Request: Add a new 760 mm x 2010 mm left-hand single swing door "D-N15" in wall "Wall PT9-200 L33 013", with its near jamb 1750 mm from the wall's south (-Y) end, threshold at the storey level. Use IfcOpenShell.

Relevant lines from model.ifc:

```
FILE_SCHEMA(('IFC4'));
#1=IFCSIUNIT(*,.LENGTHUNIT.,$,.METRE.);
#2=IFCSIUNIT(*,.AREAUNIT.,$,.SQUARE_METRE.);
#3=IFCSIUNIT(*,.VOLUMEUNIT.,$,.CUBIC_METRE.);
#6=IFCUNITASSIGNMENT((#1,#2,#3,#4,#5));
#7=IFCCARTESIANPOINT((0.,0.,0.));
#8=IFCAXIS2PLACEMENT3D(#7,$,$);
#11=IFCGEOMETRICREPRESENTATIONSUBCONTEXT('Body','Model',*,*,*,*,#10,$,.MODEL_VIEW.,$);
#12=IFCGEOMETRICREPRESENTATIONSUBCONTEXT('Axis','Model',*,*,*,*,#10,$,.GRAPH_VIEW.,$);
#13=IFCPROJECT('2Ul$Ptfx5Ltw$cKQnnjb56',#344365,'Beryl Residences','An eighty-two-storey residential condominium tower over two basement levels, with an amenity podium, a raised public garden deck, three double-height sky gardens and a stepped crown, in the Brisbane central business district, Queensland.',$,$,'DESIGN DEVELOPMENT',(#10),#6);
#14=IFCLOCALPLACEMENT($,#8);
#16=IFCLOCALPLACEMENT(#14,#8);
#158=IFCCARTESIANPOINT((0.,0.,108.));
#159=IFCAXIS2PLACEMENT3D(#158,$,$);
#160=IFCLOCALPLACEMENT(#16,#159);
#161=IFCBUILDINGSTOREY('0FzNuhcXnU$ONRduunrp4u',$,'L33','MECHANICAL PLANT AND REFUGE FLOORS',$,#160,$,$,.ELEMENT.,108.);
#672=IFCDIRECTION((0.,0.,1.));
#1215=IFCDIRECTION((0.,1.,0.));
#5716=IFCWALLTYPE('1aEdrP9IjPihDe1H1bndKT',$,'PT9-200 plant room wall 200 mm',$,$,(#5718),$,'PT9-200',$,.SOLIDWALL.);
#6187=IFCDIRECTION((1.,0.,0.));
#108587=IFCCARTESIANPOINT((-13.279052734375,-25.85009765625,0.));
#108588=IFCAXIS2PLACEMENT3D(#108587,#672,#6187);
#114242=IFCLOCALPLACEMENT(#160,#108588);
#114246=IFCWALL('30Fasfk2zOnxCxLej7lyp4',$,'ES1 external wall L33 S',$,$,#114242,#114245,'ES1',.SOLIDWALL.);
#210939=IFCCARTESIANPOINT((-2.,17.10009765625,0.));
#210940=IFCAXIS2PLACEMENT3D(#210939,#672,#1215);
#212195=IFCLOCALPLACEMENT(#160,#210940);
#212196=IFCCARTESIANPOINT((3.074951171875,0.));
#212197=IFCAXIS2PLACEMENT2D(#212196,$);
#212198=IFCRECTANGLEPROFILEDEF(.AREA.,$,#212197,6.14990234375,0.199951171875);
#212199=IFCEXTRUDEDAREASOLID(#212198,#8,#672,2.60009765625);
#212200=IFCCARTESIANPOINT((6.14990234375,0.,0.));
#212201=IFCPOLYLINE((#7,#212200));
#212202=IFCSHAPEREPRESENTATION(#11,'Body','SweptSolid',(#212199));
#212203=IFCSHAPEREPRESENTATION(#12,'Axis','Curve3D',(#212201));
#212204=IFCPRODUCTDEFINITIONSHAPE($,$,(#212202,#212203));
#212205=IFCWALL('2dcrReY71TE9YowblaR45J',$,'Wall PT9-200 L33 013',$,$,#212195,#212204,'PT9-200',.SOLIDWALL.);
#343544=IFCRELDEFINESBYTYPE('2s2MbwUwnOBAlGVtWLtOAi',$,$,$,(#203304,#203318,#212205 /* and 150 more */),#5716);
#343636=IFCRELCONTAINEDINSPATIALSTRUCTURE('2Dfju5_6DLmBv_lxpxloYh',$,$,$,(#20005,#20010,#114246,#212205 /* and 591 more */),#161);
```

```python
import numpy as np
import ifcopenshell
import ifcopenshell.api.feature
import ifcopenshell.api.geometry
import ifcopenshell.api.root
import ifcopenshell.api.spatial
import ifcopenshell.geom
import ifcopenshell.util.element
import ifcopenshell.util.placement
import ifcopenshell.util.representation
import ifcopenshell.util.shape
import ifcopenshell.util.unit

model = ifcopenshell.open("model.ifc")
unit_scale = ifcopenshell.util.unit.calculate_unit_scale(model)
settings = ifcopenshell.geom.settings()


def volume(element):
    """Net volume in cubic metres, openings subtracted."""
    shape = ifcopenshell.geom.create_shape(settings, element)
    return ifcopenshell.util.shape.get_volume(shape.geometry)


wall = model.by_guid("2dcrReY71TE9YowblaR45J")
storey = ifcopenshell.util.element.get_container(wall, ifc_class="IfcBuildingStorey")
context = ifcopenshell.util.representation.get_context(model, "Model", "Body", "MODEL_VIEW")
before = volume(wall)

width, height, from_end, sill = 0.76, 2.01, 1.75, 0.0  # metres

# The wall runs along its own X axis, and the end named is its -X end.
wall_shape = ifcopenshell.geom.create_shape(settings, wall)
x, y, z = ifcopenshell.util.shape.get_vertices(wall_shape.geometry).T
start = x.min() + from_end
face, thickness = float(y.min()), float(y.max() - y.min())
wall_matrix = ifcopenshell.util.placement.get_local_placement(wall.ObjectPlacement)
level = ifcopenshell.util.placement.get_local_placement(storey.ObjectPlacement)[2, 3]


def in_wall(x, y):
    """Placement at x, y metres in the wall's axes, at sill height."""
    matrix = wall_matrix.copy()
    matrix[:, 3] = wall_matrix @ np.array([x / unit_scale, y / unit_scale, 0.0, 1.0])
    matrix[2, 3] = level + sill / unit_scale
    return matrix


# Opening: a box that overshoots both wall faces by 50 mm.
opening = ifcopenshell.api.root.create_entity(model, ifc_class="IfcOpeningElement", predefined_type="OPENING")
box = ifcopenshell.api.geometry.add_wall_representation(
    model, context=context, length=width, height=height, thickness=thickness + 0.1
)
ifcopenshell.api.geometry.assign_representation(model, product=opening, representation=box)
ifcopenshell.api.geometry.edit_object_placement(model, product=opening, matrix=in_wall(start, face - 0.05), is_si=False)
ifcopenshell.api.feature.add_feature(model, feature=opening, element=wall)

door = ifcopenshell.api.root.create_entity(model, ifc_class="IfcDoor", name="D-N15", predefined_type="DOOR")
door.OverallWidth, door.OverallHeight = width / unit_scale, height / unit_scale
door.OperationType = "SINGLE_SWING_LEFT"
body = ifcopenshell.api.geometry.add_door_representation(
    model,
    context=context,
    overall_width=door.OverallWidth,
    overall_height=door.OverallHeight,
    operation_type="SINGLE_SWING_LEFT",
    lining_properties={"LiningDepth": thickness / unit_scale, "ThresholdDepth": thickness / unit_scale},
)
ifcopenshell.api.geometry.assign_representation(model, product=door, representation=body)
ifcopenshell.api.spatial.assign_container(model, products=[door], relating_structure=storey)
ifcopenshell.api.feature.add_filling(model, opening=opening, element=door)

# The lining spans the wall, so the door starts at the wall face.
ifcopenshell.api.geometry.edit_object_placement(model, product=door, matrix=in_wall(start, face), is_si=False)

after = volume(wall)

print(f"wall volume {before:.3f} -> {after:.3f} m3")

model.write("model_v2.ifc")
```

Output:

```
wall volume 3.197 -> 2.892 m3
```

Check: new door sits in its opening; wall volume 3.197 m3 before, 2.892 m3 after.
